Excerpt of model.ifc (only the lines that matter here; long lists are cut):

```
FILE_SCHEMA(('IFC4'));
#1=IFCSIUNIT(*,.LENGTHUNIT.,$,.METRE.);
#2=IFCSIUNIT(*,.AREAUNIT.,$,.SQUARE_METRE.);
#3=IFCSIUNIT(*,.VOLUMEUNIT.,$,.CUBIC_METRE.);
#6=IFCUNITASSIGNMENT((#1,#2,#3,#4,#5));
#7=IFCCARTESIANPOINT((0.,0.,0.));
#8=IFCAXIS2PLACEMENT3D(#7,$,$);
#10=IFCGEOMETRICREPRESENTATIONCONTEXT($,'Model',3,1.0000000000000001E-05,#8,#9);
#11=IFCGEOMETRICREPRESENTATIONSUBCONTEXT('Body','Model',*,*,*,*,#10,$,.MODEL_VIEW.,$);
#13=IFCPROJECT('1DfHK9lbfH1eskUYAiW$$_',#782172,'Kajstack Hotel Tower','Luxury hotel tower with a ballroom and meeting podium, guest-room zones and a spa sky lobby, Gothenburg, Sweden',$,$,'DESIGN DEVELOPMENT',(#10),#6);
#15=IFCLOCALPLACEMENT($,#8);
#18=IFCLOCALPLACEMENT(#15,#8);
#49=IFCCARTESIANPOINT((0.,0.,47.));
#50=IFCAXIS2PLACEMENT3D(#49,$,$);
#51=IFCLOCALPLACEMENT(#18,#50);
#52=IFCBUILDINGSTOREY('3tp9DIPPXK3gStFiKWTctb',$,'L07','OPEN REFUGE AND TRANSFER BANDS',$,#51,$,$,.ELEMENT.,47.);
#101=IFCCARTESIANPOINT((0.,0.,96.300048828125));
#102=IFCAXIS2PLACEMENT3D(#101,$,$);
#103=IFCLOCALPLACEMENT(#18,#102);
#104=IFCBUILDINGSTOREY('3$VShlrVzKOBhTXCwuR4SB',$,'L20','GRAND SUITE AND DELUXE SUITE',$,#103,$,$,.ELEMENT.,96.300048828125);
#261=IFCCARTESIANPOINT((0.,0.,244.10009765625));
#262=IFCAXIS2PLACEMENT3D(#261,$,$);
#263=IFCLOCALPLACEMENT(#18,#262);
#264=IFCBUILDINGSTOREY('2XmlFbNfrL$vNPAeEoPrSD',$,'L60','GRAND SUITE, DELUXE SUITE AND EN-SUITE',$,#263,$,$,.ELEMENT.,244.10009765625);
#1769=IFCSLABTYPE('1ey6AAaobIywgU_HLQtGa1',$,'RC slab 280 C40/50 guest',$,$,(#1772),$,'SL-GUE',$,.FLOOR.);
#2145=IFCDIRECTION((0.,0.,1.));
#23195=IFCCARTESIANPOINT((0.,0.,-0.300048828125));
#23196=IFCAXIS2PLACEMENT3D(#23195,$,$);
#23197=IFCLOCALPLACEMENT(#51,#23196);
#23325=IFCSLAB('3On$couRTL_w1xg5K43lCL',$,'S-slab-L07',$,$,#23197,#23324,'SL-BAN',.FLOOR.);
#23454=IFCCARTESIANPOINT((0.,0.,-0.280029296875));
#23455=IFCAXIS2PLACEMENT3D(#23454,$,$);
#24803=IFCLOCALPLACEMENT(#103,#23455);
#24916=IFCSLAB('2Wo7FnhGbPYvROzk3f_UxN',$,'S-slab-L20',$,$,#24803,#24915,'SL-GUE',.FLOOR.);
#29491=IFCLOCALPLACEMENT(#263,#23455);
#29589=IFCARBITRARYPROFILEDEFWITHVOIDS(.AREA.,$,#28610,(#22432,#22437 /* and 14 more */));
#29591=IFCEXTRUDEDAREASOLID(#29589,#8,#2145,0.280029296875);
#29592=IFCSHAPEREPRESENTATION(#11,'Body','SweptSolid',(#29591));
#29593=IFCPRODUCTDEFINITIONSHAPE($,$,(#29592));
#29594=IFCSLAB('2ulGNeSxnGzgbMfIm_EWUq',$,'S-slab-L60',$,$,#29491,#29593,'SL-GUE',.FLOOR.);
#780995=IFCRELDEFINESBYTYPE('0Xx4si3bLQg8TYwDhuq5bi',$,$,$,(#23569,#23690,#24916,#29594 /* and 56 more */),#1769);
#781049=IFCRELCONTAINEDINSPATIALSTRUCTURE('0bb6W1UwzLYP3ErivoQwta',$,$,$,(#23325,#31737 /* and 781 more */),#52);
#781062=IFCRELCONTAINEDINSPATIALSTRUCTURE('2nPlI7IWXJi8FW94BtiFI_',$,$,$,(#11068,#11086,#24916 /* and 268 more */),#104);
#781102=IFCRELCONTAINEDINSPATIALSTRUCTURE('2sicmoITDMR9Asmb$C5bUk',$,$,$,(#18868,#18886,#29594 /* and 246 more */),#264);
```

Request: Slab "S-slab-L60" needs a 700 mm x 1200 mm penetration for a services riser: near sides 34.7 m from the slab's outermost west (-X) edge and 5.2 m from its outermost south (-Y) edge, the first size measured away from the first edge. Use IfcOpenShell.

```python
import numpy as np
import ifcopenshell
import ifcopenshell.api.feature
import ifcopenshell.api.geometry
import ifcopenshell.api.root
import ifcopenshell.geom
import ifcopenshell.util.placement
import ifcopenshell.util.representation
import ifcopenshell.util.shape
import ifcopenshell.util.unit

model = ifcopenshell.open("model.ifc")
unit_scale = ifcopenshell.util.unit.calculate_unit_scale(model)
settings = ifcopenshell.geom.settings()


def volume(element):
    """Net volume in cubic metres, openings subtracted."""
    shape = ifcopenshell.geom.create_shape(settings, element)
    return ifcopenshell.util.shape.get_volume(shape.geometry)


slab = model.by_guid("2ulGNeSxnGzgbMfIm_EWUq")
before = volume(slab)

# Extent in the slab's own axes, in metres. The edges named are its -X and -Y sides.
slab_shape = ifcopenshell.geom.create_shape(settings, slab)
vertices = ifcopenshell.util.shape.get_vertices(slab_shape.geometry)
x_min, y_min, bottom = vertices.min(axis=0)
top = vertices[:, 2].max()

opening = ifcopenshell.api.root.create_entity(model, ifc_class="IfcOpeningElement", name="Services riser opening", predefined_type="OPENING")
context = ifcopenshell.util.representation.get_context(model, "Model", "Body", "MODEL_VIEW")
width, depth = 0.7, 1.2
outline = [(0.0, 0.0), (width, 0.0), (width, depth), (0.0, depth), (0.0, 0.0)]
# Overshoot both faces by 50 mm so the cut is clean.
shape = ifcopenshell.api.geometry.add_slab_representation(
    model, context=context, depth=top - bottom + 0.1, polyline=outline
)
ifcopenshell.api.geometry.assign_representation(model, product=opening, representation=shape)

matrix = ifcopenshell.util.placement.get_local_placement(slab.ObjectPlacement)
matrix[:, 3] = matrix @ np.append(np.array([x_min + 34.7, y_min + 5.2, bottom - 0.05]) / unit_scale, 1.0)
ifcopenshell.api.geometry.edit_object_placement(model, product=opening, matrix=matrix, is_si=False)
ifcopenshell.api.feature.add_feature(model, feature=opening, element=slab)

after = volume(slab)

print(f"slab volume {before:.3f} -> {after:.3f} m3")

model.write("model_rev.ifc")
```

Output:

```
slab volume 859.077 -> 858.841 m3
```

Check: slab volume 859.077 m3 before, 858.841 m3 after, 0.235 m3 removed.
